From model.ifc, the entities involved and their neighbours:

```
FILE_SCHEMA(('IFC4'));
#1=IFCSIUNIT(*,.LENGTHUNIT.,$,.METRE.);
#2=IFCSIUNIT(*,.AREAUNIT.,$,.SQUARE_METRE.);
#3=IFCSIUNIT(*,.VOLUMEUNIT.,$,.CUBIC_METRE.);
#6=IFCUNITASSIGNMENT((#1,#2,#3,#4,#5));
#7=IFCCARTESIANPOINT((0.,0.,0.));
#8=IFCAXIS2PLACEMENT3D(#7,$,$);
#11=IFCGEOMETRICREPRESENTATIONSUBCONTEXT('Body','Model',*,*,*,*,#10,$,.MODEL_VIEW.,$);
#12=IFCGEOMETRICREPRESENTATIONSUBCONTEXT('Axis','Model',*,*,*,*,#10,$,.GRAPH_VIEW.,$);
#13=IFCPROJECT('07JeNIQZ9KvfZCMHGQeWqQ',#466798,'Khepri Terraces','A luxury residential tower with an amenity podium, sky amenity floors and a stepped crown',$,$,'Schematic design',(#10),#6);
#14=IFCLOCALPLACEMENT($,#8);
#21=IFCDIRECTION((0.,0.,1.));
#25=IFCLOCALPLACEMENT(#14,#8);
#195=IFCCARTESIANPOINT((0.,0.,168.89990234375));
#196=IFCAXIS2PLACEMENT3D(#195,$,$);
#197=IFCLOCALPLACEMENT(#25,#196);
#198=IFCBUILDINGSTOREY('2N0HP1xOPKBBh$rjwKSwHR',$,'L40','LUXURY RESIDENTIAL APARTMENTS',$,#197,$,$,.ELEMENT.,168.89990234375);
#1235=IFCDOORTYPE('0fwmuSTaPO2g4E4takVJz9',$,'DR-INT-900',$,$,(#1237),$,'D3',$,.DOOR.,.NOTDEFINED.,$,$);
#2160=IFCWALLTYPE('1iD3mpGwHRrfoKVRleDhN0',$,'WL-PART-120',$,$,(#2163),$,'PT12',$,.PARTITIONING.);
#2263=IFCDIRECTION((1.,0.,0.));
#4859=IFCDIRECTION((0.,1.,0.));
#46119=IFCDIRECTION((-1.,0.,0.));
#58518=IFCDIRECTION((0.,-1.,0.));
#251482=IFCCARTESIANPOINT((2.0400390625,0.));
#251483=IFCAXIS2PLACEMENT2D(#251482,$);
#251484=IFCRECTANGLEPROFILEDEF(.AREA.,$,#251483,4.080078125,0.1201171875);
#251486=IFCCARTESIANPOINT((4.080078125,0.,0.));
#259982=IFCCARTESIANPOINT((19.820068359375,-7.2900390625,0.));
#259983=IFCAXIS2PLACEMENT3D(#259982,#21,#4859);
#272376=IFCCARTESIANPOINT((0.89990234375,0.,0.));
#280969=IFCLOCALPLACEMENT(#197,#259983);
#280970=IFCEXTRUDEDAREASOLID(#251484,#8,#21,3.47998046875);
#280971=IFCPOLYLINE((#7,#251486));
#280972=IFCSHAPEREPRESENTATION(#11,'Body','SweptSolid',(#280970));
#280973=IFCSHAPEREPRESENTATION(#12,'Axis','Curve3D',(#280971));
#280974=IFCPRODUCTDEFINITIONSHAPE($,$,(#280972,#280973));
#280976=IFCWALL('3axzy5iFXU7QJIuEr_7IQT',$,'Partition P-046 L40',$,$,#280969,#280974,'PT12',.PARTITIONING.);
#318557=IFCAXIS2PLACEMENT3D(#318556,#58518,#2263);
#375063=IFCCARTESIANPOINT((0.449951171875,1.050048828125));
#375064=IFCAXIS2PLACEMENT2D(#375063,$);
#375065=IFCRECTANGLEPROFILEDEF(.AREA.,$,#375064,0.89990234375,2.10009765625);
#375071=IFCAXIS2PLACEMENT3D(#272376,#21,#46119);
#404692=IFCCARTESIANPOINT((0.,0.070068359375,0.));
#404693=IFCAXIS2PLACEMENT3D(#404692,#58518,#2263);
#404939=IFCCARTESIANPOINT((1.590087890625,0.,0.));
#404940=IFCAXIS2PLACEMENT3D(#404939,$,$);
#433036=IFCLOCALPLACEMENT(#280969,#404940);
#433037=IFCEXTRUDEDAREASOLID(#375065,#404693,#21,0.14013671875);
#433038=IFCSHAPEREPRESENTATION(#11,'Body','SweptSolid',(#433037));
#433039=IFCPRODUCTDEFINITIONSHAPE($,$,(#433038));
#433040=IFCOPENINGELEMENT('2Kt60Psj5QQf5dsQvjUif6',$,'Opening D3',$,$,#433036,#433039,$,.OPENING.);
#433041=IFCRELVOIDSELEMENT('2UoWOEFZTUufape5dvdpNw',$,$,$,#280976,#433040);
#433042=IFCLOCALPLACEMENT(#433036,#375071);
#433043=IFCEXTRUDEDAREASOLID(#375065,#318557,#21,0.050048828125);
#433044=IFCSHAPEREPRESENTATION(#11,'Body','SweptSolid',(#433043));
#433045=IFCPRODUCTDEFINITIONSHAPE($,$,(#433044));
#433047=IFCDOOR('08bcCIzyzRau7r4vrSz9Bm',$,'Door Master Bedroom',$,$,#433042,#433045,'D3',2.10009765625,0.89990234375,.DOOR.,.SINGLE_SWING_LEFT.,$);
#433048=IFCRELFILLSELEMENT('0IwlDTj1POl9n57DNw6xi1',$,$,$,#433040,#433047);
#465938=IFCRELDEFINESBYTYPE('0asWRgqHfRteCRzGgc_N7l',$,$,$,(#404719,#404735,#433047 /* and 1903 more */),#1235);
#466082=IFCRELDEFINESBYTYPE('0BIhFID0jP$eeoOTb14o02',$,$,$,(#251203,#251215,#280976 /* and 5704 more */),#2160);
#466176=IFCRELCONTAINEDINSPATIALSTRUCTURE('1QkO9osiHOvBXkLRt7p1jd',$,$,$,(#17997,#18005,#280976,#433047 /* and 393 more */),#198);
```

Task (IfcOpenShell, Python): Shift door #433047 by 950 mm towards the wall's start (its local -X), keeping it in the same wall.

```python
import ifcopenshell
import ifcopenshell.api.geometry
import ifcopenshell.util.placement

model = ifcopenshell.open("model.ifc")

door = model.by_guid("08bcCIzyzRau7r4vrSz9Bm")
opening = door.FillsVoids[0].RelatingOpeningElement
wall = opening.VoidsElements[0].RelatingBuildingElement

wall_matrix = ifcopenshell.util.placement.get_local_placement(wall.ObjectPlacement)
shift = wall_matrix[:3, 0] * -0.95
before = ifcopenshell.util.placement.get_local_placement(door.ObjectPlacement)[:3, 3].copy()

# The door is placed relative to its opening, so it follows when the opening moves.
matrix = ifcopenshell.util.placement.get_local_placement(opening.ObjectPlacement)
matrix[:3, 3] += shift
ifcopenshell.api.geometry.edit_object_placement(
    model, product=opening, matrix=matrix, is_si=False, should_transform_children=True
)

after = ifcopenshell.util.placement.get_local_placement(door.ObjectPlacement)[:3, 3]
print("door moved by", (after - before).round(3) + 0.0)

model.write("model_edited.ifc")
```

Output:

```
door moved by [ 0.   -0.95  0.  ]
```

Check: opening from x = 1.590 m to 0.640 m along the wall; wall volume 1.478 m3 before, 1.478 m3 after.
